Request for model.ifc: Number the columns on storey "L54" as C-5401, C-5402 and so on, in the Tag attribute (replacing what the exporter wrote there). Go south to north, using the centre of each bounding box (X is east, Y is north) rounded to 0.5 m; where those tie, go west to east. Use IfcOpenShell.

First a look at what the model holds.

```python
import ifcopenshell
import ifcopenshell.util.element
import ifcopenshell.util.placement

model = ifcopenshell.open("model.ifc")
print(model.schema)
storey = next(s for s in model.by_type("IfcBuildingStorey") if s.Name == "L54")
columns = [e for e in ifcopenshell.util.element.get_decomposition(storey) if e.is_a("IfcColumn")]
for e in sorted(columns, key=lambda e: e.id()):
    origin = ifcopenshell.util.placement.get_local_placement(e.ObjectPlacement)[:3, 3]
    print(e.id(), e.Tag, e.Name, origin.round(2) + 0.0, sep=" | ")
```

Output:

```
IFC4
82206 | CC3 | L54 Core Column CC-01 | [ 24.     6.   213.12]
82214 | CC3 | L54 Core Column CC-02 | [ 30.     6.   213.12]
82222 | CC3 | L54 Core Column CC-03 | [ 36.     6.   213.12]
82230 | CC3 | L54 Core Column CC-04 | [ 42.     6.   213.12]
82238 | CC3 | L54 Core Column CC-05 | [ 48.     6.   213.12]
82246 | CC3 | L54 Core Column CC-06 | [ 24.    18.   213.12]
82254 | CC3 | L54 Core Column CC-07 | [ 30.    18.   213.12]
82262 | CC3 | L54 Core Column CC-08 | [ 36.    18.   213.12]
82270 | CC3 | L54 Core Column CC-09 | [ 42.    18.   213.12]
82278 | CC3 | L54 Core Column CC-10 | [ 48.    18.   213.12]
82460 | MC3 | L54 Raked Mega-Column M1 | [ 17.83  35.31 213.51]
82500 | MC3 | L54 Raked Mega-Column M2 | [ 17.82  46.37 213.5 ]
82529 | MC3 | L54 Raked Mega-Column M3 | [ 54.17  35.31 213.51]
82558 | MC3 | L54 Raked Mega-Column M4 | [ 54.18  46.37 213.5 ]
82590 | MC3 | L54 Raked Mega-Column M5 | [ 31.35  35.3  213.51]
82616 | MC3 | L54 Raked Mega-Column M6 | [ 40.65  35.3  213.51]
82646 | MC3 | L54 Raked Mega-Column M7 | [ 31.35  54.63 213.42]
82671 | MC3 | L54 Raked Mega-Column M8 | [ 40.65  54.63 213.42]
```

```python
import ifcopenshell
import ifcopenshell.geom
import ifcopenshell.util.element
import ifcopenshell.util.shape

model = ifcopenshell.open("model.ifc")
settings = ifcopenshell.geom.settings()
settings.set("use-world-coords", True)


def centre(element):
    shape = ifcopenshell.geom.create_shape(settings, element)
    return ifcopenshell.util.shape.get_bbox_centroid(shape.geometry)


storey = next(s for s in model.by_type("IfcBuildingStorey") if s.Name == "L54")
columns = [e for e in ifcopenshell.util.element.get_decomposition(storey) if e.is_a("IfcColumn")]

# Insertion points can sit at a corner or the storey origin, so sort by the geometry (in metres).
centres = {e: centre(e) for e in columns}
columns.sort(key=lambda e: (round(centres[e][1] / 0.5), centres[e][0]))

for i, e in enumerate(columns, start=1):
    number = f"C-54{i:02d}"
    e.Tag = number
    print(e.id(), number)

model.write("model_v2.ifc")
```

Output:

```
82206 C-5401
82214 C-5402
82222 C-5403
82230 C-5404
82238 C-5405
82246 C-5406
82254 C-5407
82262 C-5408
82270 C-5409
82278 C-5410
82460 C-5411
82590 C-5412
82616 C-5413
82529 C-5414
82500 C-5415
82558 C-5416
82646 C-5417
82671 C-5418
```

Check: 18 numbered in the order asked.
